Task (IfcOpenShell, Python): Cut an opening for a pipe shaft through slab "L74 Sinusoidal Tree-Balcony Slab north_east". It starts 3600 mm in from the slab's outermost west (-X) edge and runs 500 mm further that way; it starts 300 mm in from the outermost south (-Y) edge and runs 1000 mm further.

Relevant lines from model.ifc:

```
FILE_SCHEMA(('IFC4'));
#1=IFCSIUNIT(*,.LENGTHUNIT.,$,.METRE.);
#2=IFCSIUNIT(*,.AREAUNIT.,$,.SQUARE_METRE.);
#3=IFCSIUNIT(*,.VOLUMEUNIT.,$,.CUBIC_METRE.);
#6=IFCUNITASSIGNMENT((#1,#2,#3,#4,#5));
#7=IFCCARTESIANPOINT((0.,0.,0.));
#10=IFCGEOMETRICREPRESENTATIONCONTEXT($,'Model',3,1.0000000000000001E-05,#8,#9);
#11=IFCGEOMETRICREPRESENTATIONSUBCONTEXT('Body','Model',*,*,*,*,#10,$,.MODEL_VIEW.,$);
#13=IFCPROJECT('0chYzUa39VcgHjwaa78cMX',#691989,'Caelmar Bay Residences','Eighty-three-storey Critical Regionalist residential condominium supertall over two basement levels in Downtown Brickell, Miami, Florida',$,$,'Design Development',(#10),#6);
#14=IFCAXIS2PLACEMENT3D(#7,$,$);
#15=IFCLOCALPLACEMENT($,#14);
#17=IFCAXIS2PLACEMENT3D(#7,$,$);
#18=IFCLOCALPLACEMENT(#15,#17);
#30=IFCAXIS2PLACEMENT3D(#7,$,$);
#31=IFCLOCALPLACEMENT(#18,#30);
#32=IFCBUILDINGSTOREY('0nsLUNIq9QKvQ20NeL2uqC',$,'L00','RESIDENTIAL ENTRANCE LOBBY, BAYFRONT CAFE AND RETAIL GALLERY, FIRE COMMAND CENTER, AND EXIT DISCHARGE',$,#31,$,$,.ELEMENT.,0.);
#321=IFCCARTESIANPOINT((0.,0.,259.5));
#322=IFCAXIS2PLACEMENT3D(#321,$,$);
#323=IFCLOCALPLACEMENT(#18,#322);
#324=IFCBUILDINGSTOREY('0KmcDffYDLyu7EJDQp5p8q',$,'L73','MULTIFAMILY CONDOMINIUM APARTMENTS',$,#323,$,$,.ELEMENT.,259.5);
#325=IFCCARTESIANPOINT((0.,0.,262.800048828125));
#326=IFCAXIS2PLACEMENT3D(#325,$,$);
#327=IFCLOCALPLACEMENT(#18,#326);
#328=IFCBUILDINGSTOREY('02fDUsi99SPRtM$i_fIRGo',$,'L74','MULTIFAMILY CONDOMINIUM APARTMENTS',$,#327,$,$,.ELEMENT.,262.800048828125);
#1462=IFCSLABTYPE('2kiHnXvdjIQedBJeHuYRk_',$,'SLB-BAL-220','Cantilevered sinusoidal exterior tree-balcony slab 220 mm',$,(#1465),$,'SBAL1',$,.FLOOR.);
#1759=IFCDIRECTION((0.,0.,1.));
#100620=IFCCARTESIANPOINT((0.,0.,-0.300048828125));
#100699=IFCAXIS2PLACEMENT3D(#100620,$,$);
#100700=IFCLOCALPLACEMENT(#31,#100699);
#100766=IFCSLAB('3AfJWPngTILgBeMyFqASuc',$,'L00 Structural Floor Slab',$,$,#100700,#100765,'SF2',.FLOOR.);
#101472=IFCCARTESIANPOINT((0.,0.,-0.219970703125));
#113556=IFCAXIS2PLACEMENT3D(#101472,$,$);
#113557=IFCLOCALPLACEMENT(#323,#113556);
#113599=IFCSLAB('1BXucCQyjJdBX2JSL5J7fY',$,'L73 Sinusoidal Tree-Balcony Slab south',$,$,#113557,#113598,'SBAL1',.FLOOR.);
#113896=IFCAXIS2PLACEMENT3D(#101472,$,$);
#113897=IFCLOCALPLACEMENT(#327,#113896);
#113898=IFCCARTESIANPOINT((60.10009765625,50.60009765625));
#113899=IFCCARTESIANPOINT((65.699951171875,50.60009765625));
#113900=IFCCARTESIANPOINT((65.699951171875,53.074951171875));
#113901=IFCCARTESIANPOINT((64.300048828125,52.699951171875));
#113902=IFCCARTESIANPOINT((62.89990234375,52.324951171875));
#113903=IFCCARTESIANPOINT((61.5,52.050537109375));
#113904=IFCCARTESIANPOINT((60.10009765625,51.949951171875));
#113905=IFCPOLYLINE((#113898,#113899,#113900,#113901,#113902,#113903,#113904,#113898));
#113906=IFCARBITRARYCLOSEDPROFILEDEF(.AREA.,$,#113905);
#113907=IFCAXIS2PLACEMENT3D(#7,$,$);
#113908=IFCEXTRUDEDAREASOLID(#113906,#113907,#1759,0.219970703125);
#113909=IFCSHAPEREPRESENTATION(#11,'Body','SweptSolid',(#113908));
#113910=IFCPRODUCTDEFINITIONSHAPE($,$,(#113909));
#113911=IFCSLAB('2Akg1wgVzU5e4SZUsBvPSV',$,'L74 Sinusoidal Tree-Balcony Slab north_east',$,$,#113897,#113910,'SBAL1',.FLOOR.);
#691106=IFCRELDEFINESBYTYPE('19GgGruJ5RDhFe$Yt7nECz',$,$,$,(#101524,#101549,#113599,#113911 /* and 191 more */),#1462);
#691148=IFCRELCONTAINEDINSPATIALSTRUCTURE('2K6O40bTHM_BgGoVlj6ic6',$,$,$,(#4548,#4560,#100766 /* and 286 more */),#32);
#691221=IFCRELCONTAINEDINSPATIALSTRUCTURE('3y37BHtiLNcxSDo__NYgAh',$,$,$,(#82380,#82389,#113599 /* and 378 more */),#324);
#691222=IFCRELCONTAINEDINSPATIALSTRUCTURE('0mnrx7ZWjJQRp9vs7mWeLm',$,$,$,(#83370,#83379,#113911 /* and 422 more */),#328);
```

```python
import numpy as np
import ifcopenshell
import ifcopenshell.api.feature
import ifcopenshell.api.geometry
import ifcopenshell.api.root
import ifcopenshell.geom
import ifcopenshell.util.placement
import ifcopenshell.util.representation
import ifcopenshell.util.shape
import ifcopenshell.util.unit

model = ifcopenshell.open("model.ifc")
unit_scale = ifcopenshell.util.unit.calculate_unit_scale(model)
settings = ifcopenshell.geom.settings()


def volume(element):
    """Net volume in cubic metres, openings subtracted."""
    shape = ifcopenshell.geom.create_shape(settings, element)
    return ifcopenshell.util.shape.get_volume(shape.geometry)


slab = model.by_guid("2Akg1wgVzU5e4SZUsBvPSV")
before = volume(slab)

# Extent in the slab's own axes, in metres. The edges named are its -X and -Y sides.
slab_shape = ifcopenshell.geom.create_shape(settings, slab)
vertices = ifcopenshell.util.shape.get_vertices(slab_shape.geometry)
x_min, y_min, bottom = vertices.min(axis=0)
top = vertices[:, 2].max()

opening = ifcopenshell.api.root.create_entity(model, ifc_class="IfcOpeningElement", name="Pipe shaft opening", predefined_type="OPENING")
context = ifcopenshell.util.representation.get_context(model, "Model", "Body", "MODEL_VIEW")
width, depth = 0.5, 1
outline = [(0.0, 0.0), (width, 0.0), (width, depth), (0.0, depth), (0.0, 0.0)]
# Overshoot both faces by 50 mm so the cut is clean.
shape = ifcopenshell.api.geometry.add_slab_representation(
    model, context=context, depth=top - bottom + 0.1, polyline=outline
)
ifcopenshell.api.geometry.assign_representation(model, product=opening, representation=shape)

matrix = ifcopenshell.util.placement.get_local_placement(slab.ObjectPlacement)
matrix[:, 3] = matrix @ np.append(np.array([x_min + 3.6, y_min + 0.3, bottom - 0.05]) / unit_scale, 1.0)
ifcopenshell.api.geometry.edit_object_placement(model, product=opening, matrix=matrix, is_si=False)
ifcopenshell.api.feature.add_feature(model, feature=opening, element=slab)

after = volume(slab)

print(f"slab volume {before:.3f} -> {after:.3f} m3")

model.write("model_updated.ifc")
```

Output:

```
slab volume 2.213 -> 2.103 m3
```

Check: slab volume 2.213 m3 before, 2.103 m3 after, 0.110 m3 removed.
